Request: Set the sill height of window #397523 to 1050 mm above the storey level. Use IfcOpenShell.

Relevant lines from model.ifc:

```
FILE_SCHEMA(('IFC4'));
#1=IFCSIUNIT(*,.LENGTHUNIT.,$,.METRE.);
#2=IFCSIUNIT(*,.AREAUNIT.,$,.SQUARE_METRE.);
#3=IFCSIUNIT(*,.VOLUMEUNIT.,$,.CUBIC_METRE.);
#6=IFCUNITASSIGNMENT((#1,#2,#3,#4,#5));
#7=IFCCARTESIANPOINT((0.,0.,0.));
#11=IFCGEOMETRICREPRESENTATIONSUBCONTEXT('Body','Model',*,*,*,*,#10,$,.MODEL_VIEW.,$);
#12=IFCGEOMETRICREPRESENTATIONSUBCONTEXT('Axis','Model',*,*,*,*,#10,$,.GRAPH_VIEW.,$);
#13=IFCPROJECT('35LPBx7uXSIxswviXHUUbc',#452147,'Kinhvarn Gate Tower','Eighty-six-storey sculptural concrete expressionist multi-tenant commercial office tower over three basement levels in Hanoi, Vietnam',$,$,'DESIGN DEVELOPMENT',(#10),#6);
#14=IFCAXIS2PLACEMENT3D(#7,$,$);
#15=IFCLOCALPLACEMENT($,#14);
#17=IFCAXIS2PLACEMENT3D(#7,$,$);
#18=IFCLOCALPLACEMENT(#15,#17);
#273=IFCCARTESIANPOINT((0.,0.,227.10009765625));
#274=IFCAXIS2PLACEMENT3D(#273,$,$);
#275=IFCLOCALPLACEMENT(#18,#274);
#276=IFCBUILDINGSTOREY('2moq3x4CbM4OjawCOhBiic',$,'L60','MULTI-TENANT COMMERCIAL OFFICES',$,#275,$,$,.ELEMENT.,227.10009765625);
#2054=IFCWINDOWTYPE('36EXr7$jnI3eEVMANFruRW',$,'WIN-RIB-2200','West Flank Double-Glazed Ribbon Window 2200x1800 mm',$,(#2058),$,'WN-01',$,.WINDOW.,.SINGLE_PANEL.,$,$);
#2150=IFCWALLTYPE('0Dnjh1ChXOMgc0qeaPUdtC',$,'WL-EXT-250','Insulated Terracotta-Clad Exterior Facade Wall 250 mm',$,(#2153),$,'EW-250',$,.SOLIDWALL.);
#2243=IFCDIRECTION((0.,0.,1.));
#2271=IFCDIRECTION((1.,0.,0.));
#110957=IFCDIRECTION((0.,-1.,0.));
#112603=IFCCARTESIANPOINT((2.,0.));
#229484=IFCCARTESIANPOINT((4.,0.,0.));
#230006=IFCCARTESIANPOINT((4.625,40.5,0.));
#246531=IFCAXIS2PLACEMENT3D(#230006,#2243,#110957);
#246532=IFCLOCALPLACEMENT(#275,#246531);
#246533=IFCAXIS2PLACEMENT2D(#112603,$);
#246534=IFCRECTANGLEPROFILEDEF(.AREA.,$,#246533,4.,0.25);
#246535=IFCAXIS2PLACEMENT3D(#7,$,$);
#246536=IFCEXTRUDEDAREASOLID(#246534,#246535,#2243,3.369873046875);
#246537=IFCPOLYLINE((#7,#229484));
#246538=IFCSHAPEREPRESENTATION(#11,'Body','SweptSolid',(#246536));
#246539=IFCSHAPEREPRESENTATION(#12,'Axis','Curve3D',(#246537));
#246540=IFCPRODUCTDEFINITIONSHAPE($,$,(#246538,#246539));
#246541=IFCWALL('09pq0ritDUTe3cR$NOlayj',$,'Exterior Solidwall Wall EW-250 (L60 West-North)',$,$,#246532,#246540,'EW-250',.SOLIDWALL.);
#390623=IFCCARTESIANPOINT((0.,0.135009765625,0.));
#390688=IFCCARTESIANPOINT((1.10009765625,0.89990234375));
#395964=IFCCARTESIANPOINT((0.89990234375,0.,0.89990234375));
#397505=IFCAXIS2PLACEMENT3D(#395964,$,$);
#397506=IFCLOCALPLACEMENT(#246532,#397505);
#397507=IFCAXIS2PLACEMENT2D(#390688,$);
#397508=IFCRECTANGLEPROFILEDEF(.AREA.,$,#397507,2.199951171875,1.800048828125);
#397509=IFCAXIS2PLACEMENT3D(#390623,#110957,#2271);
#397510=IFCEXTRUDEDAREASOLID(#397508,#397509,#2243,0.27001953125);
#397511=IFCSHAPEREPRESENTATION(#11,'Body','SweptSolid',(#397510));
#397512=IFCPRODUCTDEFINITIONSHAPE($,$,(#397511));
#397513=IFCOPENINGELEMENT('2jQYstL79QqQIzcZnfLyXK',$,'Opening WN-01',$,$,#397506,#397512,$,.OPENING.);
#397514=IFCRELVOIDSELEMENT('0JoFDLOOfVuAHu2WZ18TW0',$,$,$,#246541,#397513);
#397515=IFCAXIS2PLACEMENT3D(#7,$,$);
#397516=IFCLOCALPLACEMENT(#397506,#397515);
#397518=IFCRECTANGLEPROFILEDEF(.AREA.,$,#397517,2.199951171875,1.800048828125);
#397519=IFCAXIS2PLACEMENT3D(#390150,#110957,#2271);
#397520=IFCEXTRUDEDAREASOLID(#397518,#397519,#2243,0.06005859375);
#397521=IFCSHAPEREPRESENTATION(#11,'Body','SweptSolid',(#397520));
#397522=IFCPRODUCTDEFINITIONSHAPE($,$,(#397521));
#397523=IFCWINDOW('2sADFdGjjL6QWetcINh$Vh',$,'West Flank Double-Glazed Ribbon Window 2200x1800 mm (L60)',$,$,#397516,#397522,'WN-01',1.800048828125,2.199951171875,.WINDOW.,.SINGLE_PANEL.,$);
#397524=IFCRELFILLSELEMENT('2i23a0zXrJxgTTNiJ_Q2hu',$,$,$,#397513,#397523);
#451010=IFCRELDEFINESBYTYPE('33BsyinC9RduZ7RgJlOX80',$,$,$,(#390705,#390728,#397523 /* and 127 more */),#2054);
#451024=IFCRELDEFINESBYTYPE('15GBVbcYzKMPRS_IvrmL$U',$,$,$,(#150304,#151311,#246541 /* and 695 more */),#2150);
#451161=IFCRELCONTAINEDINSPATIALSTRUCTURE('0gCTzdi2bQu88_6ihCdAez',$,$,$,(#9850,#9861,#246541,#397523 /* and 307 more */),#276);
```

```python
import numpy as np
import ifcopenshell
import ifcopenshell.api.geometry
import ifcopenshell.geom
import ifcopenshell.util.element
import ifcopenshell.util.placement
import ifcopenshell.util.shape
import ifcopenshell.util.unit

model = ifcopenshell.open("model.ifc")
unit_scale = ifcopenshell.util.unit.calculate_unit_scale(model)

window = model.by_id(397523)
opening = window.FillsVoids[0].RelatingOpeningElement
storey = ifcopenshell.util.element.get_container(window, ifc_class="IfcBuildingStorey")
level = ifcopenshell.util.placement.get_local_placement(storey.ObjectPlacement)[2, 3]

# The opening's origin need not be at the sill, so measure its lowest point.
shape = ifcopenshell.geom.create_shape(ifcopenshell.geom.settings(), opening)
bottom = ifcopenshell.util.shape.get_shape_bottom_elevation(shape, shape.geometry) / unit_scale
dz = level + 1.05 / unit_scale - bottom

shift = np.array([0.0, 0.0, dz])
# The window is placed relative to its opening, so it follows when the opening moves.
matrix = ifcopenshell.util.placement.get_local_placement(opening.ObjectPlacement)
matrix[:3, 3] += shift
ifcopenshell.api.geometry.edit_object_placement(
    model, product=opening, matrix=matrix, is_si=False, should_transform_children=True
)

print(f"moved by {dz * unit_scale:+.3f} m")

model.write("model-out.ifc")
```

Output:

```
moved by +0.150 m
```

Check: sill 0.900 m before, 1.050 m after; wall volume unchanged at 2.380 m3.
